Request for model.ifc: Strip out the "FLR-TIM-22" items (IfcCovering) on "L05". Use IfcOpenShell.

First a look at what the model holds.

```python
import ifcopenshell
import ifcopenshell.util.element

model = ifcopenshell.open("model.ifc")
print(model.schema)
storey = next(s for s in model.by_type("IfcBuildingStorey") if s.Name == "L05")
coverings = [e for e in ifcopenshell.util.element.get_decomposition(storey) if e.is_a("IfcCovering")]
seen = {}
for e in coverings:
    element_type = ifcopenshell.util.element.get_type(e)
    name = element_type.Name if element_type not in (None, e) else None
    seen[name] = seen.get(name, 0) + 1
for name, count in sorted(seen.items(), key=str):
    print(count, "x", name)
```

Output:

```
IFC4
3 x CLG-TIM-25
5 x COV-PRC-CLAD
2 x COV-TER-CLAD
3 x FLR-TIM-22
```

```python
import ifcopenshell
import ifcopenshell.api.root
import ifcopenshell.util.element

model = ifcopenshell.open("model.ifc")

storey = next(s for s in model.by_type("IfcBuildingStorey") if s.Name == "L05")
coverings = [e for e in ifcopenshell.util.element.get_decomposition(storey) if e.is_a("IfcCovering")]
targets = [e for e in coverings if (t := ifcopenshell.util.element.get_type(e)) not in (None, e) and t.Name == "FLR-TIM-22"]

for e in targets:
    ifcopenshell.api.root.remove_product(model, product=e)
print(len(targets), "removed")

model.write("model_rev.ifc")
```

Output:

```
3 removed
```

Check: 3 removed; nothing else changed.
